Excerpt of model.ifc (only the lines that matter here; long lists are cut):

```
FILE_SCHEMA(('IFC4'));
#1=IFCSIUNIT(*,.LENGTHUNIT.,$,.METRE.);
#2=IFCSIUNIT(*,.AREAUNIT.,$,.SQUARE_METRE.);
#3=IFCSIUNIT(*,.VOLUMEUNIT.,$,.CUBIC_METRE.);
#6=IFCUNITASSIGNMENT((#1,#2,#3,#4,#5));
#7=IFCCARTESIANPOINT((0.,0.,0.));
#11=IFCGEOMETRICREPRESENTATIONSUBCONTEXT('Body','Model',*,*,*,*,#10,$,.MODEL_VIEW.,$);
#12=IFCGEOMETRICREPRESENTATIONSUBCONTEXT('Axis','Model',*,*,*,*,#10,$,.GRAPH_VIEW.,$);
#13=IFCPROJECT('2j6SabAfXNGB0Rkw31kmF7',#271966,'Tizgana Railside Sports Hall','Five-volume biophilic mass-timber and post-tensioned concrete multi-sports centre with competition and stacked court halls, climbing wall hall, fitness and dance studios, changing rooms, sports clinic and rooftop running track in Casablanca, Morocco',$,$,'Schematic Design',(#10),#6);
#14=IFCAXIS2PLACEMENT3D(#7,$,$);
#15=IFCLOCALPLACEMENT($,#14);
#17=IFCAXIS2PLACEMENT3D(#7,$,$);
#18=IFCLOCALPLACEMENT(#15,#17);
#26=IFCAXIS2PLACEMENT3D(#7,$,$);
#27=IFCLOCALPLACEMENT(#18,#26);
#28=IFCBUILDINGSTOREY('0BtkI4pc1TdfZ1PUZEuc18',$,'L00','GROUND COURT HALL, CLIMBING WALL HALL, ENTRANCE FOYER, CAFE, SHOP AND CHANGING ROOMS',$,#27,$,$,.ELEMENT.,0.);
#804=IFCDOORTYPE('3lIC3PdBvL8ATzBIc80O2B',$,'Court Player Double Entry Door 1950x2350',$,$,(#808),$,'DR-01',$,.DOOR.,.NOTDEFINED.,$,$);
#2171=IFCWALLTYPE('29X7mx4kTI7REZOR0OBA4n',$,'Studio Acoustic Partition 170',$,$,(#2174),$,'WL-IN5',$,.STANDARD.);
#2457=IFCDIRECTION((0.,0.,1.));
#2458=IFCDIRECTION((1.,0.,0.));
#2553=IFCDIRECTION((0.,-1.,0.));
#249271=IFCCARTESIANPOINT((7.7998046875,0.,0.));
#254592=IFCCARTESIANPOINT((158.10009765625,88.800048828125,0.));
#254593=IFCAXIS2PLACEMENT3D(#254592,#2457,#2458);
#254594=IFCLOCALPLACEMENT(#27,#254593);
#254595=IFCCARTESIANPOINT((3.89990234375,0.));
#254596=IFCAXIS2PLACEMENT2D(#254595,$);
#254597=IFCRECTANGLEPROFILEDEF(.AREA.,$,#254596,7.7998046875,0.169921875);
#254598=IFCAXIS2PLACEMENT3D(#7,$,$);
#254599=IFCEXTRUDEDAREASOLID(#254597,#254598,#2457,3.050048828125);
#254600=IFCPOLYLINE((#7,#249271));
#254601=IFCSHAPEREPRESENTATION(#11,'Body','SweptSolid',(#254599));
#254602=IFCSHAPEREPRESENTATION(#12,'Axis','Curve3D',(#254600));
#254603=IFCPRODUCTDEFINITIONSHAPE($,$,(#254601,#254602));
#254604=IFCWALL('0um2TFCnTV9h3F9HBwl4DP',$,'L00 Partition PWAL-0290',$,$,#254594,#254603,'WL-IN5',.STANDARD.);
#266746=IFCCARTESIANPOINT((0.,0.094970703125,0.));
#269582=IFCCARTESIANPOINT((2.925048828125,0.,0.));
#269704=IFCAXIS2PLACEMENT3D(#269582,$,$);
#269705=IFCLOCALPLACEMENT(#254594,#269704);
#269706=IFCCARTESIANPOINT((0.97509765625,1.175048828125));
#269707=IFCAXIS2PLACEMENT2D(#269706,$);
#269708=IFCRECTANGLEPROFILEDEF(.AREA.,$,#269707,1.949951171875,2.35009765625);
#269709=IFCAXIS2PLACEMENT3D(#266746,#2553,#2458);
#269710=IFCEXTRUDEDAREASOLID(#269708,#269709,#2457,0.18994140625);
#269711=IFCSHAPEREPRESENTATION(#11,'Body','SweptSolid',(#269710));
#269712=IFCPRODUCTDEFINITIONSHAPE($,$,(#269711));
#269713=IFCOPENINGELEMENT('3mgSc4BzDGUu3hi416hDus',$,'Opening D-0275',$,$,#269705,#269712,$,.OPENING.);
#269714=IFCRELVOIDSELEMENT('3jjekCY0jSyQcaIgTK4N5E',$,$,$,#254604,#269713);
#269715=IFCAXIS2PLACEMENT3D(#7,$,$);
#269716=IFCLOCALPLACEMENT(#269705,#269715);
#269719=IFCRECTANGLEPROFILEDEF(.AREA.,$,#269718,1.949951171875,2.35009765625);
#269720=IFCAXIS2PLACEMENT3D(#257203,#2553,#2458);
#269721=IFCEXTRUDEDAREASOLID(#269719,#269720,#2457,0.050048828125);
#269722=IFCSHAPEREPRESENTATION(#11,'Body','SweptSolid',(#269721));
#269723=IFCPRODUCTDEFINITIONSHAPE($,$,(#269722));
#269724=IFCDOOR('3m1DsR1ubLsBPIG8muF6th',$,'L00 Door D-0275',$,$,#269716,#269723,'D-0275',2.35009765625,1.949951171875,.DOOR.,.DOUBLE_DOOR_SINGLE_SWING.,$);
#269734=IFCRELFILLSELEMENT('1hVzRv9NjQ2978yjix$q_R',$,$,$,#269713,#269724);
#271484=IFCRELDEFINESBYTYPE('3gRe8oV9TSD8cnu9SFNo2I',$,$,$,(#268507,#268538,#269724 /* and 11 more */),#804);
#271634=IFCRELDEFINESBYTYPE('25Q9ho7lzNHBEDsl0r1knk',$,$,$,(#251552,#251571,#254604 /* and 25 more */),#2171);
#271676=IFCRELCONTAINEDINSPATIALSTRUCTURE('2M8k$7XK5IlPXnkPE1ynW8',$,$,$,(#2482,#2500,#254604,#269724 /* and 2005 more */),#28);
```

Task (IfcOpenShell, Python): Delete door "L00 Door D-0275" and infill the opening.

```python
import ifcopenshell
import ifcopenshell.api.feature
import ifcopenshell.api.root
import ifcopenshell.geom
import ifcopenshell.util.shape

model = ifcopenshell.open("model.ifc")
settings = ifcopenshell.geom.settings()


def volume(element):
    """Net volume in cubic metres, openings subtracted."""
    shape = ifcopenshell.geom.create_shape(settings, element)
    return ifcopenshell.util.shape.get_volume(shape.geometry)


door = model.by_guid("3m1DsR1ubLsBPIG8muF6th")
opening = door.FillsVoids[0].RelatingOpeningElement
wall = opening.VoidsElements[0].RelatingBuildingElement
before = volume(wall)

ifcopenshell.api.root.remove_product(model, product=door)
ifcopenshell.api.feature.remove_feature(model, feature=opening)

after = volume(wall)

print(f"wall volume {before:.3f} -> {after:.3f} m3")

model.write("model_rev.ifc")
```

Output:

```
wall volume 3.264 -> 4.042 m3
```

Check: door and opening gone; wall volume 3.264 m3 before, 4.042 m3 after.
